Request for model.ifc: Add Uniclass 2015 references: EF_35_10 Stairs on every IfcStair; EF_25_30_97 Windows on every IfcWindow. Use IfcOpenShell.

First a look at what the model holds.

```python
import ifcopenshell

model = ifcopenshell.open("model.ifc")
print(model.schema)
print("classifications:", [c.Name for c in model.by_type("IfcClassification")])
for ifc_class in ("IfcDoor", "IfcRoof", "IfcStair", "IfcWall", "IfcWindow"):
    print(ifc_class, len(model.by_type(ifc_class)))
```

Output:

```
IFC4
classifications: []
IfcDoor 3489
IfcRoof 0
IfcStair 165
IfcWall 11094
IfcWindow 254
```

```python
import ifcopenshell
import ifcopenshell.api.classification

model = ifcopenshell.open("model.ifc")

system = ifcopenshell.api.classification.add_classification(model, classification="Uniclass 2015")

codes = {
    "IfcStair": ("EF_35_10", "Stairs"),
    "IfcWindow": ("EF_25_30_97", "Windows"),
}
for ifc_class, (code, name) in codes.items():
    products = model.by_type(ifc_class)
    ifcopenshell.api.classification.add_reference(
        model, products=products, classification=system, identification=code, name=name
    )
    print(code, len(products))

model.write("model_v2.ifc")
```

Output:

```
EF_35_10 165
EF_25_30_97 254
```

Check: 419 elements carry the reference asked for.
